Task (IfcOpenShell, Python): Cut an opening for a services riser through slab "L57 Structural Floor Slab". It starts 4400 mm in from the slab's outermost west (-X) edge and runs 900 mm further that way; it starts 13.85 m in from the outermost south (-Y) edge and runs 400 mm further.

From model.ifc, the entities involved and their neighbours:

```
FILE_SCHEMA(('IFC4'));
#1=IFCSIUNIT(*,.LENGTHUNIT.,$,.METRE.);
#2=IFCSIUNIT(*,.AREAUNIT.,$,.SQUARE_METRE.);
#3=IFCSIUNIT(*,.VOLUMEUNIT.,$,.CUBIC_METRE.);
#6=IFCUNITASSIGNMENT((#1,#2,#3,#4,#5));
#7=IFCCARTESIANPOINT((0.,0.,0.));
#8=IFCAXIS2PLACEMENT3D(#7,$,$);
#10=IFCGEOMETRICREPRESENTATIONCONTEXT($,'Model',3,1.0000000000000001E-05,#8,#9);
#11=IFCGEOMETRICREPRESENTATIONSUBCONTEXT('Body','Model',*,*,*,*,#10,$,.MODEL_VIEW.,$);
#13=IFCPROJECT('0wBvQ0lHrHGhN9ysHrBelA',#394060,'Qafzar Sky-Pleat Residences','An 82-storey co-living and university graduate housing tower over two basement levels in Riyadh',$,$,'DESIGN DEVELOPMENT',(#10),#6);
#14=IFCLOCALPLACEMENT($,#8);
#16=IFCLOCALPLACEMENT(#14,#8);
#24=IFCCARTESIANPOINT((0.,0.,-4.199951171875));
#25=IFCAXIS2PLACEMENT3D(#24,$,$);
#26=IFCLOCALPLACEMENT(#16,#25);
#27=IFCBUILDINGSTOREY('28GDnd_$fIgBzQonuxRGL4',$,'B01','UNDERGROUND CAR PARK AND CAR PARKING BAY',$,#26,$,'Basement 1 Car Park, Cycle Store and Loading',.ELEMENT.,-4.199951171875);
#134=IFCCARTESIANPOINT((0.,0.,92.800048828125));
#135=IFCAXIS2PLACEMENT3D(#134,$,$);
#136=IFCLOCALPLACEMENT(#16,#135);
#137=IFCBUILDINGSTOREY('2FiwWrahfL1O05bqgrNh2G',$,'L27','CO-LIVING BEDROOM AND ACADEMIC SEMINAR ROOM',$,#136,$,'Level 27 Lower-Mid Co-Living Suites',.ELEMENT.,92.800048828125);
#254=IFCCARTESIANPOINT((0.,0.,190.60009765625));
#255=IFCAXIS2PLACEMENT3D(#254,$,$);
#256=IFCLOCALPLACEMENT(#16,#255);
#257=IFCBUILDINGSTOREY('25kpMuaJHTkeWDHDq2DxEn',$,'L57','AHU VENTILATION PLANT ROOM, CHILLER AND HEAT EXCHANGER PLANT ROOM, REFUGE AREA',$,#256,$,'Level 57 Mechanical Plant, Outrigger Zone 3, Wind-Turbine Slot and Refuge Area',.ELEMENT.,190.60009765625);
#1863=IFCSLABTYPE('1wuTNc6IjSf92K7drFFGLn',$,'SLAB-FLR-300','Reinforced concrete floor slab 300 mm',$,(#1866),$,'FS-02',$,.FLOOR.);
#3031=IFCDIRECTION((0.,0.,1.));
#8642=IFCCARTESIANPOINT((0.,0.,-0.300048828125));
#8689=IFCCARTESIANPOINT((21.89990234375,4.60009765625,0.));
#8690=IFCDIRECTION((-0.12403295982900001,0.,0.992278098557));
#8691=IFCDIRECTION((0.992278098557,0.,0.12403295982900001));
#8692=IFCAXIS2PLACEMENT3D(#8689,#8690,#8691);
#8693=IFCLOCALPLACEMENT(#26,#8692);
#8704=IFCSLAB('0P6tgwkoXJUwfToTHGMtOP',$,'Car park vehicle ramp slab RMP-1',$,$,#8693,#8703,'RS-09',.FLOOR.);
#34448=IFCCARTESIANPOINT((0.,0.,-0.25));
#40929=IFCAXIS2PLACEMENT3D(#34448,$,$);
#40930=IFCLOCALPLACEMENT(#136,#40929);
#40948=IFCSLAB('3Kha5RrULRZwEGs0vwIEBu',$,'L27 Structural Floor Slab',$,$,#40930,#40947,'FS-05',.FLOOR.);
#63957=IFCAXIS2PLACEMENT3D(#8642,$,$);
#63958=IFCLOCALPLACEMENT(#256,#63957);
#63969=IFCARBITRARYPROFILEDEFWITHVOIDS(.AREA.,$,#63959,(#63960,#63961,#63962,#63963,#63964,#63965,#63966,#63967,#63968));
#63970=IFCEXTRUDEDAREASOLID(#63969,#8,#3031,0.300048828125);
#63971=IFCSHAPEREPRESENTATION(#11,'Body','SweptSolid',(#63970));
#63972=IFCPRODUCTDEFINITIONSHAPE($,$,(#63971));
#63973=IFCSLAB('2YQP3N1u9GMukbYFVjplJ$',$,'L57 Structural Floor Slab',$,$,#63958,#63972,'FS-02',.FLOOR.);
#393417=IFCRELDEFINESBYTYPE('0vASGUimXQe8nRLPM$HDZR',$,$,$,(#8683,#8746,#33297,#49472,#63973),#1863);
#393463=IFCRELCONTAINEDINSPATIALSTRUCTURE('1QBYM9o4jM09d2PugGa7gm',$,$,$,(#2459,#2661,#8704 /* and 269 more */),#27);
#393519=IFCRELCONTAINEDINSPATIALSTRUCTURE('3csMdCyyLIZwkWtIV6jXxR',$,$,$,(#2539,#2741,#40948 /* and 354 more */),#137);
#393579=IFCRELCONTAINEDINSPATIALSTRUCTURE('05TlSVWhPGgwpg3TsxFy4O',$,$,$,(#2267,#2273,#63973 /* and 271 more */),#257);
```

```python
import numpy as np
import ifcopenshell
import ifcopenshell.api.feature
import ifcopenshell.api.geometry
import ifcopenshell.api.root
import ifcopenshell.geom
import ifcopenshell.util.placement
import ifcopenshell.util.representation
import ifcopenshell.util.shape
import ifcopenshell.util.unit

model = ifcopenshell.open("model.ifc")
unit_scale = ifcopenshell.util.unit.calculate_unit_scale(model)
settings = ifcopenshell.geom.settings()


def volume(element):
    """Net volume in cubic metres, openings subtracted."""
    shape = ifcopenshell.geom.create_shape(settings, element)
    return ifcopenshell.util.shape.get_volume(shape.geometry)


slab = model.by_guid("2YQP3N1u9GMukbYFVjplJ$")
before = volume(slab)

# Extent in the slab's own axes, in metres. The edges named are its -X and -Y sides.
slab_shape = ifcopenshell.geom.create_shape(settings, slab)
vertices = ifcopenshell.util.shape.get_vertices(slab_shape.geometry)
x_min, y_min, bottom = vertices.min(axis=0)
top = vertices[:, 2].max()

opening = ifcopenshell.api.root.create_entity(model, ifc_class="IfcOpeningElement", name="Services riser opening", predefined_type="OPENING")
context = ifcopenshell.util.representation.get_context(model, "Model", "Body", "MODEL_VIEW")
width, depth = 0.9, 0.4
outline = [(0.0, 0.0), (width, 0.0), (width, depth), (0.0, depth), (0.0, 0.0)]
# Overshoot both faces by 50 mm so the cut is clean.
shape = ifcopenshell.api.geometry.add_slab_representation(
    model, context=context, depth=top - bottom + 0.1, polyline=outline
)
ifcopenshell.api.geometry.assign_representation(model, product=opening, representation=shape)

matrix = ifcopenshell.util.placement.get_local_placement(slab.ObjectPlacement)
matrix[:, 3] = matrix @ np.append(np.array([x_min + 4.4, y_min + 13.85, bottom - 0.05]) / unit_scale, 1.0)
ifcopenshell.api.geometry.edit_object_placement(model, product=opening, matrix=matrix, is_si=False)
ifcopenshell.api.feature.add_feature(model, feature=opening, element=slab)

after = volume(slab)

print(f"slab volume {before:.3f} -> {after:.3f} m3")

model.write("model_rev.ifc")
```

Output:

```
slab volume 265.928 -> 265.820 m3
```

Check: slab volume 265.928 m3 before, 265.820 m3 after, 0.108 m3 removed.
